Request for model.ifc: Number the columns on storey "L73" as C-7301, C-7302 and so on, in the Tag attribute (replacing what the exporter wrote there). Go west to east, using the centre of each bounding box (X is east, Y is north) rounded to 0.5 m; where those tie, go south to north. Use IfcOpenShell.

First a look at what the model holds.

```python
import ifcopenshell
import ifcopenshell.util.element
import ifcopenshell.util.placement

model = ifcopenshell.open("model.ifc")
print(model.schema)
storey = next(s for s in model.by_type("IfcBuildingStorey") if s.Name == "L73")
columns = [e for e in ifcopenshell.util.element.get_decomposition(storey) if e.is_a("IfcColumn")]
for e in sorted(columns, key=lambda e: e.id()):
    origin = ifcopenshell.util.placement.get_local_placement(e.ObjectPlacement)[:3, 3]
    print(e.id(), e.Tag, e.Name, origin.round(2) + 0.0, sep=" | ")
```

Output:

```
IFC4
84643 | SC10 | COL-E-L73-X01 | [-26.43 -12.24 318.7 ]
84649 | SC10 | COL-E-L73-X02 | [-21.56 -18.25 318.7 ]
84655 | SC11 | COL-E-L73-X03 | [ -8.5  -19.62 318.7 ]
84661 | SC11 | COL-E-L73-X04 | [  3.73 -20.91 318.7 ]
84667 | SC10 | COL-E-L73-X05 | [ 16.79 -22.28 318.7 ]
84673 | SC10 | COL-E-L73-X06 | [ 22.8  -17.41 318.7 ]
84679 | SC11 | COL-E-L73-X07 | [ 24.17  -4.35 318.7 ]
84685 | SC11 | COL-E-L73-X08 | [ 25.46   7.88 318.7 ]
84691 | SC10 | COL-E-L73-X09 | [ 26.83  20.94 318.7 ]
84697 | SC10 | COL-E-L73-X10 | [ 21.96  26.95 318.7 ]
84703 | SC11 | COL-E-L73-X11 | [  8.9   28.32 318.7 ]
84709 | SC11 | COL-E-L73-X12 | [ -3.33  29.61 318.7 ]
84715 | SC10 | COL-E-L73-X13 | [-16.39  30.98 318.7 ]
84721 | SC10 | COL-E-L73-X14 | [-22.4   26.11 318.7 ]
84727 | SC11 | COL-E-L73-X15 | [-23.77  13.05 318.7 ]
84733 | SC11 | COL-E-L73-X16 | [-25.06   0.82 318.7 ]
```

```python
import ifcopenshell
import ifcopenshell.geom
import ifcopenshell.util.element
import ifcopenshell.util.shape

model = ifcopenshell.open("model.ifc")
settings = ifcopenshell.geom.settings()
settings.set("use-world-coords", True)


def centre(element):
    shape = ifcopenshell.geom.create_shape(settings, element)
    return ifcopenshell.util.shape.get_bbox_centroid(shape.geometry)


storey = next(s for s in model.by_type("IfcBuildingStorey") if s.Name == "L73")
columns = [e for e in ifcopenshell.util.element.get_decomposition(storey) if e.is_a("IfcColumn")]

# Insertion points can sit at a corner or the storey origin, so sort by the geometry (in metres).
centres = {e: centre(e) for e in columns}
columns.sort(key=lambda e: (round(centres[e][0] / 0.5), centres[e][1]))

for i, e in enumerate(columns, start=1):
    number = f"C-73{i:02d}"
    e.Tag = number
    print(e.id(), number)

model.write("model-out.ifc")
```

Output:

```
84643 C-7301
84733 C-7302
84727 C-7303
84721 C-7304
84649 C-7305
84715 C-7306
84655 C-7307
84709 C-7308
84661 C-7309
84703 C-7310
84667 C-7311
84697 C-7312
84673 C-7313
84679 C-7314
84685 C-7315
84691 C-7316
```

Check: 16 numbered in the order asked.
